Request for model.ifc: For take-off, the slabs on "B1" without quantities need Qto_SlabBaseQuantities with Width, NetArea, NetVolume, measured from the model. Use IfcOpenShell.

First a look at what the model holds.

```python
import ifcopenshell
import ifcopenshell.util.element
import ifcopenshell.util.unit

model = ifcopenshell.open("model.ifc")
print(model.schema)
for unit_type in ("LENGTHUNIT", "AREAUNIT", "VOLUMEUNIT"):
    print(unit_type, ifcopenshell.util.unit.calculate_unit_scale(model, unit_type))
storey = next(s for s in model.by_type("IfcBuildingStorey") if s.Name == "B1")
slabs = [e for e in ifcopenshell.util.element.get_decomposition(storey) if e.is_a("IfcSlab")]
for e in sorted(slabs, key=lambda e: e.id()):
    print(e.id(), e.is_a(), e.Name, list(ifcopenshell.util.element.get_psets(e, qtos_only=True)), sep=" | ")
```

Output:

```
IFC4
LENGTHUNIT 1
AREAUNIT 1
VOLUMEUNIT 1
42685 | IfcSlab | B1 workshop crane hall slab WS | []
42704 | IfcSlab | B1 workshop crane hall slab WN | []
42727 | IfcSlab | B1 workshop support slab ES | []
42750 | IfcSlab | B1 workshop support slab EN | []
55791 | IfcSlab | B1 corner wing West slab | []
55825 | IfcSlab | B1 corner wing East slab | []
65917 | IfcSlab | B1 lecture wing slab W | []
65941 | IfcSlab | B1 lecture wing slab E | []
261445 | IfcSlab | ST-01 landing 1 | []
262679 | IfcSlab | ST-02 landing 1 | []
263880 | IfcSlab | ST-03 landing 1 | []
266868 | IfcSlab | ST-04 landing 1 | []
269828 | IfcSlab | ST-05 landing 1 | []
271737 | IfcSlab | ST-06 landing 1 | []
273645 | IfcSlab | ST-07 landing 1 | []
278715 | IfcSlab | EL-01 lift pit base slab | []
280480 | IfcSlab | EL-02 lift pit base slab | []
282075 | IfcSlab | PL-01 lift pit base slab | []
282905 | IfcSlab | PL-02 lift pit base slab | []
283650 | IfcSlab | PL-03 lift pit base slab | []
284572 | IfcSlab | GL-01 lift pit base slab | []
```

```python
import ifcopenshell
import ifcopenshell.api.pset
import ifcopenshell.geom
import ifcopenshell.util.element
import ifcopenshell.util.shape
import ifcopenshell.util.unit

model = ifcopenshell.open("model.ifc")
unit_scale = ifcopenshell.util.unit.calculate_unit_scale(model)
area_scale = ifcopenshell.util.unit.calculate_unit_scale(model, "AREAUNIT")
volume_scale = ifcopenshell.util.unit.calculate_unit_scale(model, "VOLUMEUNIT")
settings = ifcopenshell.geom.settings()

storey = next(s for s in model.by_type("IfcBuildingStorey") if s.Name == "B1")
slabs = [e for e in ifcopenshell.util.element.get_decomposition(storey) if e.is_a("IfcSlab")]

for e in sorted(slabs, key=lambda e: e.id()):
    if ifcopenshell.util.element.get_psets(e, qtos_only=True, should_inherit=False):
        continue
    # Geometry comes back in metres, in the element's own axes.
    shape = ifcopenshell.geom.create_shape(settings, e)
    values = {
        "Width": ifcopenshell.util.shape.get_z(shape.geometry) / unit_scale,
        "NetArea": ifcopenshell.util.shape.get_footprint_area(shape.geometry) / area_scale,
        "NetVolume": ifcopenshell.util.shape.get_volume(shape.geometry) / volume_scale,
    }
    qto = ifcopenshell.api.pset.add_qto(model, product=e, name="Qto_SlabBaseQuantities")
    ifcopenshell.api.pset.edit_qto(model, qto=qto, properties=values)
    print(e.id(), {k: round(v, 3) for k, v in values.items()})

model.write("model_edited.ifc")
```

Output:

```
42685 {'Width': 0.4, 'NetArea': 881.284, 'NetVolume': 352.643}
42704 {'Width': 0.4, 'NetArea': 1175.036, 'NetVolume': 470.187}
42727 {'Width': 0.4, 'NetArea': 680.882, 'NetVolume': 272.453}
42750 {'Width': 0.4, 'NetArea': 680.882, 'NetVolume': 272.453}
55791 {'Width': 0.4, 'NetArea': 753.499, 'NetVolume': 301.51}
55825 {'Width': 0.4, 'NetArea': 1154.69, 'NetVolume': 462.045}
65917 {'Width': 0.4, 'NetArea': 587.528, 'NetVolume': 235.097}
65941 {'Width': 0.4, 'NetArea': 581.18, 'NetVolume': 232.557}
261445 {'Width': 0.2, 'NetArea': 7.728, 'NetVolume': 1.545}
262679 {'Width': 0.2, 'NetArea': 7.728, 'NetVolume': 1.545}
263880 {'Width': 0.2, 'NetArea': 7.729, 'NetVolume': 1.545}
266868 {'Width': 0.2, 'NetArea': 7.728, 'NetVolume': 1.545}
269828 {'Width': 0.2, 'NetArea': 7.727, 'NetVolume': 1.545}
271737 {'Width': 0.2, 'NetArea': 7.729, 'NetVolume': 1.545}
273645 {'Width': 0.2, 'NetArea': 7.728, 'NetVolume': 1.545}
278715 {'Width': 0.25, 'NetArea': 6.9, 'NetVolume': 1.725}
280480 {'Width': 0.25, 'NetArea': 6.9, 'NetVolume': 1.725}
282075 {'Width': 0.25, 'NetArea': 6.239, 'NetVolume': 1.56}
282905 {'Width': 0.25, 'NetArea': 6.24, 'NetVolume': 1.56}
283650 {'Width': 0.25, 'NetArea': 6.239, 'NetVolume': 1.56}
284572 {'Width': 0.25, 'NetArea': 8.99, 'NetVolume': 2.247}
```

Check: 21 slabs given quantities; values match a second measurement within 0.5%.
